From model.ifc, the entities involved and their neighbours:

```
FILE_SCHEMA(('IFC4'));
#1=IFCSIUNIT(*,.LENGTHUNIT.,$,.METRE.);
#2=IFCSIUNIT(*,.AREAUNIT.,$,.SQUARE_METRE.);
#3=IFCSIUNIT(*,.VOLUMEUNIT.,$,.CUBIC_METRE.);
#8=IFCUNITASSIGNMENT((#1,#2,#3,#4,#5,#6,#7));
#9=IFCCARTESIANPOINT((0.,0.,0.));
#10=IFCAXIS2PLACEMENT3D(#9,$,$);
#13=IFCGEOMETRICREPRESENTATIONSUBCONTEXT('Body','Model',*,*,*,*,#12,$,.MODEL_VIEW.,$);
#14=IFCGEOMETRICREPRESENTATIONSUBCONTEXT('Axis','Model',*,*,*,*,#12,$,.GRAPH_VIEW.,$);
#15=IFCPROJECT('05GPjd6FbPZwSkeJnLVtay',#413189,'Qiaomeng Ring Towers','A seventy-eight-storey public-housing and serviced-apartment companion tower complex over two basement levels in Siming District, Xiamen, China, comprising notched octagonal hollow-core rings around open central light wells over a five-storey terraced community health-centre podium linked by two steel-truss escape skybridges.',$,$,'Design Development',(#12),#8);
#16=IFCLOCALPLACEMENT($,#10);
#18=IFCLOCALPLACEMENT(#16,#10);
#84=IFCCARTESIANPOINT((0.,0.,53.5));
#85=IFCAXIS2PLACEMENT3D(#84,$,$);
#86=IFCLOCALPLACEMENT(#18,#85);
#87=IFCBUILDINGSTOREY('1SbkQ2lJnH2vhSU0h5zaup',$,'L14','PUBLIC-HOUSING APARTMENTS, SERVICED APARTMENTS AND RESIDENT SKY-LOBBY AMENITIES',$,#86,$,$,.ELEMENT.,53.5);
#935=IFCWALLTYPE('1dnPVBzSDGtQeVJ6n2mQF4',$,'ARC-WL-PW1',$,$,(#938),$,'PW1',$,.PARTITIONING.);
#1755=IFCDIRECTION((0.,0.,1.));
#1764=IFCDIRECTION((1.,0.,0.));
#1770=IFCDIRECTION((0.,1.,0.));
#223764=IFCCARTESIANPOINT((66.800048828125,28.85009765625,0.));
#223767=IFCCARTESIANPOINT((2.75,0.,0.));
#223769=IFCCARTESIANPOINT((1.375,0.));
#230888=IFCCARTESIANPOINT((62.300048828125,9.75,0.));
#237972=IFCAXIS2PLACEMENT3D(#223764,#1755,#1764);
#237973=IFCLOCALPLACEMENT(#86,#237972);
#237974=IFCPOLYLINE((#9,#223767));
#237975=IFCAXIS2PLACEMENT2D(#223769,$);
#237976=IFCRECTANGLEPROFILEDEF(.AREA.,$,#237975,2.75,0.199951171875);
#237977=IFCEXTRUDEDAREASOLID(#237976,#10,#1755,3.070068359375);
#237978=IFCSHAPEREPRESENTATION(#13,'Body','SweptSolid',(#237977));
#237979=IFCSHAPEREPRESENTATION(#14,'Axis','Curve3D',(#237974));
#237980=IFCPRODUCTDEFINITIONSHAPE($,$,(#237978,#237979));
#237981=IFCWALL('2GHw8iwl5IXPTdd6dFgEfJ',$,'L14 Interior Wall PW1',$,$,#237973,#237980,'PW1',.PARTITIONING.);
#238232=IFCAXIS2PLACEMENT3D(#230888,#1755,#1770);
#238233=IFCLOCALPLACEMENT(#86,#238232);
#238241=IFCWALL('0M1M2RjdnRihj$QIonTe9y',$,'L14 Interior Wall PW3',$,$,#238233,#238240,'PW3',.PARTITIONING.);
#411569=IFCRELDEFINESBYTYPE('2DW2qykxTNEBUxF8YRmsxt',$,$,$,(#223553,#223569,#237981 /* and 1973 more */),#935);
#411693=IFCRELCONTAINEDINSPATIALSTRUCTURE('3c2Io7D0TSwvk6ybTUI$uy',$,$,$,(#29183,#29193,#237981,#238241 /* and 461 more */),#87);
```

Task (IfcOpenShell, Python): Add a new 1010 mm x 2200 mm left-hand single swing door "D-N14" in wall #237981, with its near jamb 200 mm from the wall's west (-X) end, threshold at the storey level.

```python
import numpy as np
import ifcopenshell
import ifcopenshell.api.feature
import ifcopenshell.api.geometry
import ifcopenshell.api.root
import ifcopenshell.api.spatial
import ifcopenshell.geom
import ifcopenshell.util.element
import ifcopenshell.util.placement
import ifcopenshell.util.representation
import ifcopenshell.util.shape
import ifcopenshell.util.unit

model = ifcopenshell.open("model.ifc")
unit_scale = ifcopenshell.util.unit.calculate_unit_scale(model)
settings = ifcopenshell.geom.settings()


def volume(element):
    """Net volume in cubic metres, openings subtracted."""
    shape = ifcopenshell.geom.create_shape(settings, element)
    return ifcopenshell.util.shape.get_volume(shape.geometry)


wall = model.by_guid("2GHw8iwl5IXPTdd6dFgEfJ")
storey = ifcopenshell.util.element.get_container(wall, ifc_class="IfcBuildingStorey")
context = ifcopenshell.util.representation.get_context(model, "Model", "Body", "MODEL_VIEW")
before = volume(wall)

width, height, from_end, sill = 1.01, 2.2, 0.2, 0.0  # metres

# The wall runs along its own X axis, and the end named is its -X end.
wall_shape = ifcopenshell.geom.create_shape(settings, wall)
x, y, z = ifcopenshell.util.shape.get_vertices(wall_shape.geometry).T
start = x.min() + from_end
face, thickness = float(y.min()), float(y.max() - y.min())
wall_matrix = ifcopenshell.util.placement.get_local_placement(wall.ObjectPlacement)
level = ifcopenshell.util.placement.get_local_placement(storey.ObjectPlacement)[2, 3]


def in_wall(x, y):
    """Placement at x, y metres in the wall's axes, at sill height."""
    matrix = wall_matrix.copy()
    matrix[:, 3] = wall_matrix @ np.array([x / unit_scale, y / unit_scale, 0.0, 1.0])
    matrix[2, 3] = level + sill / unit_scale
    return matrix


# Opening: a box that overshoots both wall faces by 50 mm.
opening = ifcopenshell.api.root.create_entity(model, ifc_class="IfcOpeningElement", predefined_type="OPENING")
box = ifcopenshell.api.geometry.add_wall_representation(
    model, context=context, length=width, height=height, thickness=thickness + 0.1
)
ifcopenshell.api.geometry.assign_representation(model, product=opening, representation=box)
ifcopenshell.api.geometry.edit_object_placement(model, product=opening, matrix=in_wall(start, face - 0.05), is_si=False)
ifcopenshell.api.feature.add_feature(model, feature=opening, element=wall)

door = ifcopenshell.api.root.create_entity(model, ifc_class="IfcDoor", name="D-N14", predefined_type="DOOR")
door.OverallWidth, door.OverallHeight = width / unit_scale, height / unit_scale
door.OperationType = "SINGLE_SWING_LEFT"
body = ifcopenshell.api.geometry.add_door_representation(
    model,
    context=context,
    overall_width=door.OverallWidth,
    overall_height=door.OverallHeight,
    operation_type="SINGLE_SWING_LEFT",
    lining_properties={"LiningDepth": thickness / unit_scale, "ThresholdDepth": thickness / unit_scale},
)
ifcopenshell.api.geometry.assign_representation(model, product=door, representation=body)
ifcopenshell.api.spatial.assign_container(model, products=[door], relating_structure=storey)
ifcopenshell.api.feature.add_filling(model, opening=opening, element=door)

# The lining spans the wall, so the door starts at the wall face.
ifcopenshell.api.geometry.edit_object_placement(model, product=door, matrix=in_wall(start, face), is_si=False)

after = volume(wall)

print(f"wall volume {before:.3f} -> {after:.3f} m3")

model.write("model_updated.ifc")
```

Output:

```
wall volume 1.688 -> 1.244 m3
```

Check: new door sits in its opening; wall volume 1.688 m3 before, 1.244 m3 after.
